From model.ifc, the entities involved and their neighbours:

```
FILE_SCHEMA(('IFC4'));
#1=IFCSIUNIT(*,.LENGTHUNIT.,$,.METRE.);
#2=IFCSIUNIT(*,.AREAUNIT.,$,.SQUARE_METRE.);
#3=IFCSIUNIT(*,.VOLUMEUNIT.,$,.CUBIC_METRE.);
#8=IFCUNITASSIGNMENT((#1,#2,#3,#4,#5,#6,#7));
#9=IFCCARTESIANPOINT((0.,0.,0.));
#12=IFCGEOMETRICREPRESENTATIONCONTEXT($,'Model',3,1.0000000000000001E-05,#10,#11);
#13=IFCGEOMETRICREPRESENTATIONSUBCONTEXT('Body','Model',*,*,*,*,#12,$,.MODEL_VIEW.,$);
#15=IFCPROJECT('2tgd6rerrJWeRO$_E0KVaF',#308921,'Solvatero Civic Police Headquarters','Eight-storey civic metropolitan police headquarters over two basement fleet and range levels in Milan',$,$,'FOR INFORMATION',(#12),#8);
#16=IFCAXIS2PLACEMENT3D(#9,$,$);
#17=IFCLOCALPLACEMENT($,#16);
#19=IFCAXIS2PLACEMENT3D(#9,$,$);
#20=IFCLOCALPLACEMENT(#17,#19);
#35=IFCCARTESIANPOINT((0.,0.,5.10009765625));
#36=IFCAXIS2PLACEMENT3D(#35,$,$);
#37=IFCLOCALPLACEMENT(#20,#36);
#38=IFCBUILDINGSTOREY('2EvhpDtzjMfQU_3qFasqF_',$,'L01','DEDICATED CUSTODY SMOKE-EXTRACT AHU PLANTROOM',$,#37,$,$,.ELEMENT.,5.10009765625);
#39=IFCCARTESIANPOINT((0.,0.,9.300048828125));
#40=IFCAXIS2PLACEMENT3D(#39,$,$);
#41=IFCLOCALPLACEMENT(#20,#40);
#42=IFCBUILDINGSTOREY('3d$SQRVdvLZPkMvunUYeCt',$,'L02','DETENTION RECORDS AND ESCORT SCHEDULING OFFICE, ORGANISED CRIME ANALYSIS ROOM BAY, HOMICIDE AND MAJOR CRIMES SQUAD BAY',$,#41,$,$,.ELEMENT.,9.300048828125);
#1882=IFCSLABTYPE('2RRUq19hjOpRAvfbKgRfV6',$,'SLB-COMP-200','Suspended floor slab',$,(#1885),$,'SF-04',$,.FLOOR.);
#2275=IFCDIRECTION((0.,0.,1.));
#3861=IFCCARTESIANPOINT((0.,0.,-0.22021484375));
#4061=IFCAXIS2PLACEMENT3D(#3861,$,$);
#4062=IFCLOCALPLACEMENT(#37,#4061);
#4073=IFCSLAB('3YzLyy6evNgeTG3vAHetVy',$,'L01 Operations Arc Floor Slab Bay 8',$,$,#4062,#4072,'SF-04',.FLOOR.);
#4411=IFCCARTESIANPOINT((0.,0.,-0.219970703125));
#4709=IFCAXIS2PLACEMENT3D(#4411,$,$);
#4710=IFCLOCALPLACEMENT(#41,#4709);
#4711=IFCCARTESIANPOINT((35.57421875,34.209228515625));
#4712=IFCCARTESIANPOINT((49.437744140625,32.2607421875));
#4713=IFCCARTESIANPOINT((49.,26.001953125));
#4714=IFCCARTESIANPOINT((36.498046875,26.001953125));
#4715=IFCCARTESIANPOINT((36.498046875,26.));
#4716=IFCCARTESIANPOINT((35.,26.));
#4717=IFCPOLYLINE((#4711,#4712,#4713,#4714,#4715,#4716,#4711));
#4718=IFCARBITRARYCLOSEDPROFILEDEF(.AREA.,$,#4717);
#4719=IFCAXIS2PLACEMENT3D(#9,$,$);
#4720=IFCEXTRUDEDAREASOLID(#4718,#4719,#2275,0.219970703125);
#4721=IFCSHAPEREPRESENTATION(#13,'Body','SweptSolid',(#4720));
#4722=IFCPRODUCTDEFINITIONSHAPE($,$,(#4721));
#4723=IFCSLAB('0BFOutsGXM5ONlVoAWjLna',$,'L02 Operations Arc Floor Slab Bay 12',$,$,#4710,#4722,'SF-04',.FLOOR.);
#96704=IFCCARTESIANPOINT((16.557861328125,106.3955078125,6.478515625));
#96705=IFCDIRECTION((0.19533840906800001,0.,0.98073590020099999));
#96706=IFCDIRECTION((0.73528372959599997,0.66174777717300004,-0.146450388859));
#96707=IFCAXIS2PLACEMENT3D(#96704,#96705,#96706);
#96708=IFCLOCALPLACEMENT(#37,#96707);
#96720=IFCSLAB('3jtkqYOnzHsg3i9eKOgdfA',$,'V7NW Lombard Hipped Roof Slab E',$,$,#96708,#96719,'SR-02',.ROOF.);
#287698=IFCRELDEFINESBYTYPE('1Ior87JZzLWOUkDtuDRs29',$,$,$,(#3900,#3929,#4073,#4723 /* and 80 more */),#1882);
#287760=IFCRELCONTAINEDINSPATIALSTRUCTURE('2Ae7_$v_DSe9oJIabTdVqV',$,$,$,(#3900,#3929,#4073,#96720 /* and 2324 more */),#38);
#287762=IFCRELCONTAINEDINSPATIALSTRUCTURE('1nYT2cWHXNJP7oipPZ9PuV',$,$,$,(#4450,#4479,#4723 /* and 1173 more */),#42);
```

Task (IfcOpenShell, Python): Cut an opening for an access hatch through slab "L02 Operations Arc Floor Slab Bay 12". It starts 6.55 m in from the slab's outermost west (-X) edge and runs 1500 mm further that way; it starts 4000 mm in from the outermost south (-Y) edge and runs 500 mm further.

```python
import numpy as np
import ifcopenshell
import ifcopenshell.api.feature
import ifcopenshell.api.geometry
import ifcopenshell.api.root
import ifcopenshell.geom
import ifcopenshell.util.placement
import ifcopenshell.util.representation
import ifcopenshell.util.shape
import ifcopenshell.util.unit

model = ifcopenshell.open("model.ifc")
unit_scale = ifcopenshell.util.unit.calculate_unit_scale(model)
settings = ifcopenshell.geom.settings()


def volume(element):
    """Net volume in cubic metres, openings subtracted."""
    shape = ifcopenshell.geom.create_shape(settings, element)
    return ifcopenshell.util.shape.get_volume(shape.geometry)


slab = model.by_guid("0BFOutsGXM5ONlVoAWjLna")
before = volume(slab)

# Extent in the slab's own axes, in metres. The edges named are its -X and -Y sides.
slab_shape = ifcopenshell.geom.create_shape(settings, slab)
vertices = ifcopenshell.util.shape.get_vertices(slab_shape.geometry)
x_min, y_min, bottom = vertices.min(axis=0)
top = vertices[:, 2].max()

opening = ifcopenshell.api.root.create_entity(model, ifc_class="IfcOpeningElement", name="Access hatch opening", predefined_type="OPENING")
context = ifcopenshell.util.representation.get_context(model, "Model", "Body", "MODEL_VIEW")
width, depth = 1.5, 0.5
outline = [(0.0, 0.0), (width, 0.0), (width, depth), (0.0, depth), (0.0, 0.0)]
# Overshoot both faces by 50 mm so the cut is clean.
shape = ifcopenshell.api.geometry.add_slab_representation(
    model, context=context, depth=top - bottom + 0.1, polyline=outline
)
ifcopenshell.api.geometry.assign_representation(model, product=opening, representation=shape)

matrix = ifcopenshell.util.placement.get_local_placement(slab.ObjectPlacement)
matrix[:, 3] = matrix @ np.append(np.array([x_min + 6.55, y_min + 4, bottom - 0.05]) / unit_scale, 1.0)
ifcopenshell.api.geometry.edit_object_placement(model, product=opening, matrix=matrix, is_si=False)
ifcopenshell.api.feature.add_feature(model, feature=opening, element=slab)

after = volume(slab)

print(f"slab volume {before:.3f} -> {after:.3f} m3")

model.write("model_updated.ifc")
```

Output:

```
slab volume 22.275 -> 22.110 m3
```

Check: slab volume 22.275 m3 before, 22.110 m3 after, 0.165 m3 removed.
